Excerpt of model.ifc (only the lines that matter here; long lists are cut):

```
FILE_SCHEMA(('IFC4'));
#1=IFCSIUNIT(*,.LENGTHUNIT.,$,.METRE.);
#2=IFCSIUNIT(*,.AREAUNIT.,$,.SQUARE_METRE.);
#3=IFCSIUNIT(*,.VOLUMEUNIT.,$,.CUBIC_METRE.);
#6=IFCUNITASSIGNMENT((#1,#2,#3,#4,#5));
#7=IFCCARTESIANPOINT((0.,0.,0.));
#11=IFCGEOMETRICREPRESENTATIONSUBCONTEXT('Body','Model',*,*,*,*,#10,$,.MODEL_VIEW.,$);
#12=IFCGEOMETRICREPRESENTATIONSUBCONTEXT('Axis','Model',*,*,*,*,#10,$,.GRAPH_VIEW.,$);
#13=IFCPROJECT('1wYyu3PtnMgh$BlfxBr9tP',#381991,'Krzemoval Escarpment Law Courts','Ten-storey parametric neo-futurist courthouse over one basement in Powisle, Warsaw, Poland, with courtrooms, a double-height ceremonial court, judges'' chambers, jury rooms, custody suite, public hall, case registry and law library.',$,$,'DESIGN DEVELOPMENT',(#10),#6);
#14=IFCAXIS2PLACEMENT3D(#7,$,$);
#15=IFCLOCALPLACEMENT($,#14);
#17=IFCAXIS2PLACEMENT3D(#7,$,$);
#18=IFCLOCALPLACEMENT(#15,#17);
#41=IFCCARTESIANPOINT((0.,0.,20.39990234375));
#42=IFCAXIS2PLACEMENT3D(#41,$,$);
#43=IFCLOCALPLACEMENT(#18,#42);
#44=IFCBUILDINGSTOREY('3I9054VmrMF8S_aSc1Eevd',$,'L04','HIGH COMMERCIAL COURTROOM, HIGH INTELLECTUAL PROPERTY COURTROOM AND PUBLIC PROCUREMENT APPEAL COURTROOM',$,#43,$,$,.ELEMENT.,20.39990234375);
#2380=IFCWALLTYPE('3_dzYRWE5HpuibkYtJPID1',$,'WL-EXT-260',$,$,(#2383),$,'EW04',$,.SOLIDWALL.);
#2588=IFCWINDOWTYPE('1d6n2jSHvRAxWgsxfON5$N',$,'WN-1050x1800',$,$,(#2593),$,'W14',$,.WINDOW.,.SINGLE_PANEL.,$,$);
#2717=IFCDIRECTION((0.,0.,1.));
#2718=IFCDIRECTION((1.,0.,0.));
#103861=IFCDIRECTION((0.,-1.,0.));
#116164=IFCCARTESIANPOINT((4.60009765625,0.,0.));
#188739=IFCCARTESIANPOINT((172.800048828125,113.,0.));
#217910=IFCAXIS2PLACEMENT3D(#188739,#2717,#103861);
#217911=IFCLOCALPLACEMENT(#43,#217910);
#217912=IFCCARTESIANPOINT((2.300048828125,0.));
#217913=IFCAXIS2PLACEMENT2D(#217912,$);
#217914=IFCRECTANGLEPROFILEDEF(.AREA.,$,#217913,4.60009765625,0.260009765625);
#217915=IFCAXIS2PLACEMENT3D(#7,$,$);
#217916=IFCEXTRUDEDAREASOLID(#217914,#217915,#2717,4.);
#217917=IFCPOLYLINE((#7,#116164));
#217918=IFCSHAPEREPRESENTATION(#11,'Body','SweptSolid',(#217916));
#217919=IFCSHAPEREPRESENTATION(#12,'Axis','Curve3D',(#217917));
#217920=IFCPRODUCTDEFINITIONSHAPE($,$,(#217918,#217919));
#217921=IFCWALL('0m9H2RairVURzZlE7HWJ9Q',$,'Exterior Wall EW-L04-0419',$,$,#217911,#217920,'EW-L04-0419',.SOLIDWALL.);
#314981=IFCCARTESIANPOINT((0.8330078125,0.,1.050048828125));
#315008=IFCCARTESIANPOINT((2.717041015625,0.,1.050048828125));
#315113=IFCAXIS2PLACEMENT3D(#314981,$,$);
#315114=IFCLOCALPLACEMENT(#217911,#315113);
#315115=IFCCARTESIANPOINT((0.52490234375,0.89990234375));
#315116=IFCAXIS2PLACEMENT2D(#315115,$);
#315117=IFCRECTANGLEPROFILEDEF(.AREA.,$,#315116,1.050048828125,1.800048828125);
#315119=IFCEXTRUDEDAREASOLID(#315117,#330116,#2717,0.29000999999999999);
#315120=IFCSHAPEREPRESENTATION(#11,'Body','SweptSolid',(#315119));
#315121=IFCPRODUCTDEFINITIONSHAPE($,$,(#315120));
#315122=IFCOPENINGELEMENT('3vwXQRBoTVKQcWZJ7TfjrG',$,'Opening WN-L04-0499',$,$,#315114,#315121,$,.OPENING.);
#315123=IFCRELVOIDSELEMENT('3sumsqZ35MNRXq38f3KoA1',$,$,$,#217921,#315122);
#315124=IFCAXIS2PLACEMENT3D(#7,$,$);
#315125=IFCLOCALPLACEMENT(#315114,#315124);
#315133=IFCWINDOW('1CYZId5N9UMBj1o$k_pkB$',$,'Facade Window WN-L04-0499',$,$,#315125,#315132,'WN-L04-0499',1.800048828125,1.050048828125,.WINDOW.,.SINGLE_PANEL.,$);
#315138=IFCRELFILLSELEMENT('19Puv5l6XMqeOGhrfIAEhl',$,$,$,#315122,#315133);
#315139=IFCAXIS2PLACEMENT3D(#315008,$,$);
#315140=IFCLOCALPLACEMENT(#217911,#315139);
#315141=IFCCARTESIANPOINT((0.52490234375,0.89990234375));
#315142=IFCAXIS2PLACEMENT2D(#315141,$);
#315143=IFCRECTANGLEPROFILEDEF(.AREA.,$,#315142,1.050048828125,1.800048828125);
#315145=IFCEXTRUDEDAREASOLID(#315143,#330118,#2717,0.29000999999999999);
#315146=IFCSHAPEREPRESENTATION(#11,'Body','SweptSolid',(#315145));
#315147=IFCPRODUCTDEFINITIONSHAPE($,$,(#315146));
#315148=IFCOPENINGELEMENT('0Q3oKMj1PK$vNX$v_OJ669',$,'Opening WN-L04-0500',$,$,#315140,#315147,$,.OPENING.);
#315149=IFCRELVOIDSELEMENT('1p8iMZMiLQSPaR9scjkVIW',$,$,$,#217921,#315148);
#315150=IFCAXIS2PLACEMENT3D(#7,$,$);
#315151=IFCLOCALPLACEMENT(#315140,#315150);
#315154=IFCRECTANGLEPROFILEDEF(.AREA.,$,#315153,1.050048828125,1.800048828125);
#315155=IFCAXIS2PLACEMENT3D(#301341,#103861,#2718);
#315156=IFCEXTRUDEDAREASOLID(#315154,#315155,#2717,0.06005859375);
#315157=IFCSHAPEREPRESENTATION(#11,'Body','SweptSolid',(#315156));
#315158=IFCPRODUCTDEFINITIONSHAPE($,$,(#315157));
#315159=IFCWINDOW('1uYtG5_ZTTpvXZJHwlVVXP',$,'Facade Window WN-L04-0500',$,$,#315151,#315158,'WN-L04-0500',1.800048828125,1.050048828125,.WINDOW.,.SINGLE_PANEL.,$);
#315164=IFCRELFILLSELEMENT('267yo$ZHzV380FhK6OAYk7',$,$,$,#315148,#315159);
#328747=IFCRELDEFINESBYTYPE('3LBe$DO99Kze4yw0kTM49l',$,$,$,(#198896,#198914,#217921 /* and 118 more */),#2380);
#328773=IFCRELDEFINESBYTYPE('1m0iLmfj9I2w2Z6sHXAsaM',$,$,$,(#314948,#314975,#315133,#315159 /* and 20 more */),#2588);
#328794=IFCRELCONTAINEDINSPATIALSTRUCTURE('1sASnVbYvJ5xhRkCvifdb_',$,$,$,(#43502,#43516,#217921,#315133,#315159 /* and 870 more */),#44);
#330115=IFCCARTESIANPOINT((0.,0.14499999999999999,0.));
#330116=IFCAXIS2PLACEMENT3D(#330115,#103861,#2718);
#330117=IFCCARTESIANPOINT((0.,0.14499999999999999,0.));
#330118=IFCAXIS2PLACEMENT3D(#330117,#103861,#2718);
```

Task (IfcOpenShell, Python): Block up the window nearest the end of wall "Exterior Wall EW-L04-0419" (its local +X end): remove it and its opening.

```python
import ifcopenshell
import ifcopenshell.api.feature
import ifcopenshell.api.root
import ifcopenshell.geom
import ifcopenshell.util.shape

model = ifcopenshell.open("model.ifc")
settings = ifcopenshell.geom.settings()


def volume(element):
    """Net volume in cubic metres, openings subtracted."""
    shape = ifcopenshell.geom.create_shape(settings, element)
    return ifcopenshell.util.shape.get_volume(shape.geometry)


window = model.by_guid("1uYtG5_ZTTpvXZJHwlVVXP")
opening = window.FillsVoids[0].RelatingOpeningElement
wall = opening.VoidsElements[0].RelatingBuildingElement
before = volume(wall)

ifcopenshell.api.root.remove_product(model, product=window)
ifcopenshell.api.feature.remove_feature(model, feature=opening)

after = volume(wall)

print(f"wall volume {before:.3f} -> {after:.3f} m3")

model.write("model_edited.ifc")
```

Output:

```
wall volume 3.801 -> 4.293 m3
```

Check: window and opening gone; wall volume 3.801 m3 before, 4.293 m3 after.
